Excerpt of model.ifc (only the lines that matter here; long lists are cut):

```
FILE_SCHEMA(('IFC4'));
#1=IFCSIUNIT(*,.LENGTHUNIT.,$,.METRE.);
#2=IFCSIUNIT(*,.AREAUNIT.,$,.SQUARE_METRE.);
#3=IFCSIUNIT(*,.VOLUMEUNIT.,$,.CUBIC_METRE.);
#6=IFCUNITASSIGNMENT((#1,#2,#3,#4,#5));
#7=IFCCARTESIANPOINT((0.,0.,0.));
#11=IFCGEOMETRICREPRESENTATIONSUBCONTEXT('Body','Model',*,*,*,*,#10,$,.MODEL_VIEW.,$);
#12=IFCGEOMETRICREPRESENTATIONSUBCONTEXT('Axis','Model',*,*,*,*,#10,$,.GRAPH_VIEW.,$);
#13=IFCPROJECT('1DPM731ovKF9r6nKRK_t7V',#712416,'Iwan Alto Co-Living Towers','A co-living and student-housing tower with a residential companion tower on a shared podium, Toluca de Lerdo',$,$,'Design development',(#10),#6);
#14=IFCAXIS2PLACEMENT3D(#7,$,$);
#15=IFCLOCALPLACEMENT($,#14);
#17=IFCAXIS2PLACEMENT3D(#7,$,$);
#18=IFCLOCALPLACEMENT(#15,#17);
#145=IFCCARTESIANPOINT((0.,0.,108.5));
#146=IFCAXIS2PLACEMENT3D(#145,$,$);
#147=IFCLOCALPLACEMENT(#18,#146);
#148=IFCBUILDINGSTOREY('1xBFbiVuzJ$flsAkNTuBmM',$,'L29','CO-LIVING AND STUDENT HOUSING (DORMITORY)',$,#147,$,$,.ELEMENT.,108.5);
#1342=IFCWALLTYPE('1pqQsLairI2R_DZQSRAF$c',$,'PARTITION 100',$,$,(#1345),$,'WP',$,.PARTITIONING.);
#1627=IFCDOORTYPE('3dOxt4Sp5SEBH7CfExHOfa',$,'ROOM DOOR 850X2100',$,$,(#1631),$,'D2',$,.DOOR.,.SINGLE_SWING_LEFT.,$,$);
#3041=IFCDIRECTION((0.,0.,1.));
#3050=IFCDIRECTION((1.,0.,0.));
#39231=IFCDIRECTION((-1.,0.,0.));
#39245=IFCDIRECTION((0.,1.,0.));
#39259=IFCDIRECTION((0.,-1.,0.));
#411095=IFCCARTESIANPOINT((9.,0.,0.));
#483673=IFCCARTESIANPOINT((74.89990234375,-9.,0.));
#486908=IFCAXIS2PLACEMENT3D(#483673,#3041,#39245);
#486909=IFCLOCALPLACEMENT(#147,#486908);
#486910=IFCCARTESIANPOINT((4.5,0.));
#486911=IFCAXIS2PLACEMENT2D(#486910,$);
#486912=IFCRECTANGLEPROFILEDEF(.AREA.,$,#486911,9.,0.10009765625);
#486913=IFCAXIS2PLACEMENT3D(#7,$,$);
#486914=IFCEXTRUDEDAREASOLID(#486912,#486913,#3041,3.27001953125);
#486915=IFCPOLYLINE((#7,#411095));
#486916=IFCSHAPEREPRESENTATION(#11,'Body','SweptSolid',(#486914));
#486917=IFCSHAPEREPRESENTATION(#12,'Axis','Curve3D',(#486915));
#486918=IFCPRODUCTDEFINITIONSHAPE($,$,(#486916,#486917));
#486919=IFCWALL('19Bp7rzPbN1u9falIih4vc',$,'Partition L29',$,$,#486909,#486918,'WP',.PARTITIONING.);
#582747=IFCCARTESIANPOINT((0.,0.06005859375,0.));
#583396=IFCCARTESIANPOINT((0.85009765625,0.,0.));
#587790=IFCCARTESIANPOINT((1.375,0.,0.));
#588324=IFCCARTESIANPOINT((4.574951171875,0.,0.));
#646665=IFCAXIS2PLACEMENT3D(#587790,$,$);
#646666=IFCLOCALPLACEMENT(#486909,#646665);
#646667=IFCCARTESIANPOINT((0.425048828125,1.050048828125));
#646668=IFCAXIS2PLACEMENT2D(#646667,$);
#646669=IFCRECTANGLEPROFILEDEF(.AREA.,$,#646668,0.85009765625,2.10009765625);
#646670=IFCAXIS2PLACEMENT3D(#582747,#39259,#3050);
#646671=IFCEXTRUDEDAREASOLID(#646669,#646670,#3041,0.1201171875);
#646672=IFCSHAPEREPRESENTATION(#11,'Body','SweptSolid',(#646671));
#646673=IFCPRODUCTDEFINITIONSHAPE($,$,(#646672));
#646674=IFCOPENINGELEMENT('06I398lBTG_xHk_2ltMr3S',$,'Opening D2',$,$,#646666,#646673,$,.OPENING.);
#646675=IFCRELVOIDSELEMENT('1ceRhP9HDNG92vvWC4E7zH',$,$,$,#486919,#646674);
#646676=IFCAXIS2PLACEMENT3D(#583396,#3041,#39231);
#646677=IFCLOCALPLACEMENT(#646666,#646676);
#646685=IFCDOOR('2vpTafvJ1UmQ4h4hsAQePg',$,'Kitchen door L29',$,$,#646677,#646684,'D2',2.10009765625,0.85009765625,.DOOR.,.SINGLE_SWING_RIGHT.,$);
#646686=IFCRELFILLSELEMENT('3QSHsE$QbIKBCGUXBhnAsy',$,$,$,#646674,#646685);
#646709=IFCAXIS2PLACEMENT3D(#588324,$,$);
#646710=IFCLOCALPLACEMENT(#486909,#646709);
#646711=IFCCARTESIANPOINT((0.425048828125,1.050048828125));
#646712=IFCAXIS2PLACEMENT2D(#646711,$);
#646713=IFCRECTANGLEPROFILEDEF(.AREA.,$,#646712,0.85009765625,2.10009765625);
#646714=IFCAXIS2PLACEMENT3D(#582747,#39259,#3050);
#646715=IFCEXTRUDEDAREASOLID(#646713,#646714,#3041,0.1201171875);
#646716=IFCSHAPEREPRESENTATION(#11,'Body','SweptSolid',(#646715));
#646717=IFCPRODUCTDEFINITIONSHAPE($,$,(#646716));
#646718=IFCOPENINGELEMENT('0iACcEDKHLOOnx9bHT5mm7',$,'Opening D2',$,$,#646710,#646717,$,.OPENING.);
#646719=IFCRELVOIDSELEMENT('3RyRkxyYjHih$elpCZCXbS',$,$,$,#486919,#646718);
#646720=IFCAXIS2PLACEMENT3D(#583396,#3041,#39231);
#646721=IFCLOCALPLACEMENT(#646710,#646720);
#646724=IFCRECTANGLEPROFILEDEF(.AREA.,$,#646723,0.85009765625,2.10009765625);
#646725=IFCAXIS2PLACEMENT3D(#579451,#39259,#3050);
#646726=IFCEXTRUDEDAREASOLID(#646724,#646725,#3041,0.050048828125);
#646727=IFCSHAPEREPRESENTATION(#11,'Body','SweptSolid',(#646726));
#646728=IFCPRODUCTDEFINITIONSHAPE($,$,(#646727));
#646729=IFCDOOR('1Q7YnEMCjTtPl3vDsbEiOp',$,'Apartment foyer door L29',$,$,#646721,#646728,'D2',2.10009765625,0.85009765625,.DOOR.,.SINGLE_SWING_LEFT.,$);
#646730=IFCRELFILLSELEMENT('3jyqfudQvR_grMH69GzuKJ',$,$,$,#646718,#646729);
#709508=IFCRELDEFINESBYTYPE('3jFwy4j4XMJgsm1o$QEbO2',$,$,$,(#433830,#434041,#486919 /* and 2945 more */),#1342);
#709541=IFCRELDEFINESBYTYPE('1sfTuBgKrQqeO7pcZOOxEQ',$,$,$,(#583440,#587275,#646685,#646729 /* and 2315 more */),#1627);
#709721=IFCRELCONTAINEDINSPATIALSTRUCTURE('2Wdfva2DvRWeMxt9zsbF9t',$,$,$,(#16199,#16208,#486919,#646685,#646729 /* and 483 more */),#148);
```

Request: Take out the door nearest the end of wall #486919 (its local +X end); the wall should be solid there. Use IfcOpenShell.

```python
import ifcopenshell
import ifcopenshell.api.feature
import ifcopenshell.api.root
import ifcopenshell.geom
import ifcopenshell.util.shape

model = ifcopenshell.open("model.ifc")
settings = ifcopenshell.geom.settings()


def volume(element):
    """Net volume in cubic metres, openings subtracted."""
    shape = ifcopenshell.geom.create_shape(settings, element)
    return ifcopenshell.util.shape.get_volume(shape.geometry)


door = model.by_guid("1Q7YnEMCjTtPl3vDsbEiOp")
opening = door.FillsVoids[0].RelatingOpeningElement
wall = opening.VoidsElements[0].RelatingBuildingElement
before = volume(wall)

ifcopenshell.api.root.remove_product(model, product=door)
ifcopenshell.api.feature.remove_feature(model, feature=opening)

after = volume(wall)

print(f"wall volume {before:.3f} -> {after:.3f} m3")

model.write("model-out.ifc")
```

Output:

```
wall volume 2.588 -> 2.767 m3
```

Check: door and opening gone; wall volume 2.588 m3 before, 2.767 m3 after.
